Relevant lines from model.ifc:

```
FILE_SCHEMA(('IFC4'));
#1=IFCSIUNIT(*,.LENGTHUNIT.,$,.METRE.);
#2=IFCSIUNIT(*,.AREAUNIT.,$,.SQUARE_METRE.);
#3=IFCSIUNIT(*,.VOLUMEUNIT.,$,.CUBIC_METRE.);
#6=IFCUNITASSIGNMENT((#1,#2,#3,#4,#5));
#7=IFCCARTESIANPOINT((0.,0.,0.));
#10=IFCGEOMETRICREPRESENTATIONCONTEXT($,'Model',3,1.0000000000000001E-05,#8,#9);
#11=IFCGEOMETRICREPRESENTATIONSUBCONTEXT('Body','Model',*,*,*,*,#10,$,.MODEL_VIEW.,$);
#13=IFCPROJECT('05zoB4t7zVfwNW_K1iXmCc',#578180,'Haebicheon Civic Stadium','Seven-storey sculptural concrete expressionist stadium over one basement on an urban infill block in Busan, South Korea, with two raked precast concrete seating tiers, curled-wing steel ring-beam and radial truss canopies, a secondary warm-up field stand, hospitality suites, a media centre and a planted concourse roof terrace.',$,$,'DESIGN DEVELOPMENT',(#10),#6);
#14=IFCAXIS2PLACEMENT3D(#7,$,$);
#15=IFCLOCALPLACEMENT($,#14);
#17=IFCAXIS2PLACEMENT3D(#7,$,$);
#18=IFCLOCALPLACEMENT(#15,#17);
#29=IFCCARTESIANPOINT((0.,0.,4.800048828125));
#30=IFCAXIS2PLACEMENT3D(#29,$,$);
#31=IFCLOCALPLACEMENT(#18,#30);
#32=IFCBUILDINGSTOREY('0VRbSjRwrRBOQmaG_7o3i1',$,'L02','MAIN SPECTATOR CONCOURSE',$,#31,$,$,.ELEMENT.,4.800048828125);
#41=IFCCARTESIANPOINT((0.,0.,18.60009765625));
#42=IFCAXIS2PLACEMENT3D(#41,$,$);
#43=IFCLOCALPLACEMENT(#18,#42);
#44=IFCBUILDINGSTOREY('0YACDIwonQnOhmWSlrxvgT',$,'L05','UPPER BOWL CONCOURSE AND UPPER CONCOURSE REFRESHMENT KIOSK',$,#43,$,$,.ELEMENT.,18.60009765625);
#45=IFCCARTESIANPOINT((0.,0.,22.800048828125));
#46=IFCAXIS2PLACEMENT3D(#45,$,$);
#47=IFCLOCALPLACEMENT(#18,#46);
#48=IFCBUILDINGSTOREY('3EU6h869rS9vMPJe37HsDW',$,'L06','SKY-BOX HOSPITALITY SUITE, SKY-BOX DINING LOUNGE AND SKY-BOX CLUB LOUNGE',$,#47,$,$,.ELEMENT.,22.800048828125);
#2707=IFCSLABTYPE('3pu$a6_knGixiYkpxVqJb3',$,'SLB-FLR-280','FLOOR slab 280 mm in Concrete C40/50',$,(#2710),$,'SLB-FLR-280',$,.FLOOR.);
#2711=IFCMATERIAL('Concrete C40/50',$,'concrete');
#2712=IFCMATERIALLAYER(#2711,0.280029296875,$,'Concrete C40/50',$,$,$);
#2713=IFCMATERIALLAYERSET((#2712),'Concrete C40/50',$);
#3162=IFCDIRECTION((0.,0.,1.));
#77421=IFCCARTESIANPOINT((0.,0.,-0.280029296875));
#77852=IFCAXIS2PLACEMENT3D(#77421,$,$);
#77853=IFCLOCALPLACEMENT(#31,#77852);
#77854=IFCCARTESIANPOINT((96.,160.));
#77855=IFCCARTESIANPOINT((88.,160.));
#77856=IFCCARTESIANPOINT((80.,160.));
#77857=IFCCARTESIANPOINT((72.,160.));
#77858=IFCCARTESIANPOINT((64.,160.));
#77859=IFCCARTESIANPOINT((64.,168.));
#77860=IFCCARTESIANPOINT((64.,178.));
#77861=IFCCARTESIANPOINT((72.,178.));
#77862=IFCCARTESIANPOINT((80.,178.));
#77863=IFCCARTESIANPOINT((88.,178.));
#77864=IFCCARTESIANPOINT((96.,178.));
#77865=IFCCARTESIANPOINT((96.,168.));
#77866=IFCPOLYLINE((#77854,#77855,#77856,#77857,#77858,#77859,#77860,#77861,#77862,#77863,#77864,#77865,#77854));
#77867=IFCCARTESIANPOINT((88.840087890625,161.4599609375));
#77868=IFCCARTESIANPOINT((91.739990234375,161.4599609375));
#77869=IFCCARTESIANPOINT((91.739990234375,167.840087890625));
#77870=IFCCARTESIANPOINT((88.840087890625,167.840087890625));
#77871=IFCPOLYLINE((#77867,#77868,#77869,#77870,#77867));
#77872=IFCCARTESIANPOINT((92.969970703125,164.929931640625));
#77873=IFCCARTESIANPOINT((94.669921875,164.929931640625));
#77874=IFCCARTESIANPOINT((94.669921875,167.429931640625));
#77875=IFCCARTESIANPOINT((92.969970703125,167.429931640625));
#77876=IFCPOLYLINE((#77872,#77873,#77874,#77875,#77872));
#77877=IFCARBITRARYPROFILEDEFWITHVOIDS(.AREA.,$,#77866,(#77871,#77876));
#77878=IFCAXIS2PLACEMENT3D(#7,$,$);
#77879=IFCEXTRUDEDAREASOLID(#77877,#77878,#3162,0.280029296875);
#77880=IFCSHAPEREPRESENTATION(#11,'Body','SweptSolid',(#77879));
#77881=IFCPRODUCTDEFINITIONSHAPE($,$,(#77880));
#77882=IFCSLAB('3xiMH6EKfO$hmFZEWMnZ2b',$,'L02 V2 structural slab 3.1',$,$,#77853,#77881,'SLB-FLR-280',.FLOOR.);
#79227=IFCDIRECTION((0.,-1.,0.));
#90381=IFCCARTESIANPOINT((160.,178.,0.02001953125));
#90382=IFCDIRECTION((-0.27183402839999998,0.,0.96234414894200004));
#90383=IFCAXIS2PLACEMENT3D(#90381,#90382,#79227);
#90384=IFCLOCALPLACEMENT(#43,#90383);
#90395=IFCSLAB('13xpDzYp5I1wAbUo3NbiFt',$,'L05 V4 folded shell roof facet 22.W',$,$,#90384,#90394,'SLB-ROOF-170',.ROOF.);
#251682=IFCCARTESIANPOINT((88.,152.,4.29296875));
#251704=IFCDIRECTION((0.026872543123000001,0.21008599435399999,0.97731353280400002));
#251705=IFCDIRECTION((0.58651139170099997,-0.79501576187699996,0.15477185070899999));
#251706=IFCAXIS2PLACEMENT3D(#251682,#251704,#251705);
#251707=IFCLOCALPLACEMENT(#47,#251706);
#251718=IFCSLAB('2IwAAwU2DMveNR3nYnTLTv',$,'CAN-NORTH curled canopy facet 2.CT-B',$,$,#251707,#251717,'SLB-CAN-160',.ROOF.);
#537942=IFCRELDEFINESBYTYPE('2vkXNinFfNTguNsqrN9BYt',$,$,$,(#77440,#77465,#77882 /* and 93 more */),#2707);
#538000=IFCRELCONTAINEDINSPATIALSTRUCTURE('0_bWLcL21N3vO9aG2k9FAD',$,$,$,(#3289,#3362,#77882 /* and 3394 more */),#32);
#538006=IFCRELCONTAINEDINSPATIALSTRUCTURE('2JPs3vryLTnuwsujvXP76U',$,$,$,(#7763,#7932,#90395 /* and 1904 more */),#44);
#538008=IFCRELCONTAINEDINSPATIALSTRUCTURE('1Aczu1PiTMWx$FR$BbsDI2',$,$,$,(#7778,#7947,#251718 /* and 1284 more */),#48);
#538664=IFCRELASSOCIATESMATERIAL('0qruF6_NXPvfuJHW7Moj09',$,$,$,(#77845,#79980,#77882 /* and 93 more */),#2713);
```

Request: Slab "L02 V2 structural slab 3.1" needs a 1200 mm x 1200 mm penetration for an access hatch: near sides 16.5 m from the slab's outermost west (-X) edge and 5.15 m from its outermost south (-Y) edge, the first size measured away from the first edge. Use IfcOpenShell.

```python
import numpy as np
import ifcopenshell
import ifcopenshell.api.feature
import ifcopenshell.api.geometry
import ifcopenshell.api.root
import ifcopenshell.geom
import ifcopenshell.util.placement
import ifcopenshell.util.representation
import ifcopenshell.util.shape
import ifcopenshell.util.unit

model = ifcopenshell.open("model.ifc")
unit_scale = ifcopenshell.util.unit.calculate_unit_scale(model)
settings = ifcopenshell.geom.settings()


def volume(element):
    """Net volume in cubic metres, openings subtracted."""
    shape = ifcopenshell.geom.create_shape(settings, element)
    return ifcopenshell.util.shape.get_volume(shape.geometry)


slab = model.by_guid("3xiMH6EKfO$hmFZEWMnZ2b")
before = volume(slab)

# Extent in the slab's own axes, in metres. The edges named are its -X and -Y sides.
slab_shape = ifcopenshell.geom.create_shape(settings, slab)
vertices = ifcopenshell.util.shape.get_vertices(slab_shape.geometry)
x_min, y_min, bottom = vertices.min(axis=0)
top = vertices[:, 2].max()

opening = ifcopenshell.api.root.create_entity(model, ifc_class="IfcOpeningElement", name="Access hatch opening", predefined_type="OPENING")
context = ifcopenshell.util.representation.get_context(model, "Model", "Body", "MODEL_VIEW")
width, depth = 1.2, 1.2
outline = [(0.0, 0.0), (width, 0.0), (width, depth), (0.0, depth), (0.0, 0.0)]
# Overshoot both faces by 50 mm so the cut is clean.
shape = ifcopenshell.api.geometry.add_slab_representation(
    model, context=context, depth=top - bottom + 0.1, polyline=outline
)
ifcopenshell.api.geometry.assign_representation(model, product=opening, representation=shape)

matrix = ifcopenshell.util.placement.get_local_placement(slab.ObjectPlacement)
matrix[:, 3] = matrix @ np.append(np.array([x_min + 16.5, y_min + 5.15, bottom - 0.05]) / unit_scale, 1.0)
ifcopenshell.api.geometry.edit_object_placement(model, product=opening, matrix=matrix, is_si=False)
ifcopenshell.api.feature.add_feature(model, feature=opening, element=slab)

after = volume(slab)

print(f"slab volume {before:.3f} -> {after:.3f} m3")

model.write("model-out.ifc")
```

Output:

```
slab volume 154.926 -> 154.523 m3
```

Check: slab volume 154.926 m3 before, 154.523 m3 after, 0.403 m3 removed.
